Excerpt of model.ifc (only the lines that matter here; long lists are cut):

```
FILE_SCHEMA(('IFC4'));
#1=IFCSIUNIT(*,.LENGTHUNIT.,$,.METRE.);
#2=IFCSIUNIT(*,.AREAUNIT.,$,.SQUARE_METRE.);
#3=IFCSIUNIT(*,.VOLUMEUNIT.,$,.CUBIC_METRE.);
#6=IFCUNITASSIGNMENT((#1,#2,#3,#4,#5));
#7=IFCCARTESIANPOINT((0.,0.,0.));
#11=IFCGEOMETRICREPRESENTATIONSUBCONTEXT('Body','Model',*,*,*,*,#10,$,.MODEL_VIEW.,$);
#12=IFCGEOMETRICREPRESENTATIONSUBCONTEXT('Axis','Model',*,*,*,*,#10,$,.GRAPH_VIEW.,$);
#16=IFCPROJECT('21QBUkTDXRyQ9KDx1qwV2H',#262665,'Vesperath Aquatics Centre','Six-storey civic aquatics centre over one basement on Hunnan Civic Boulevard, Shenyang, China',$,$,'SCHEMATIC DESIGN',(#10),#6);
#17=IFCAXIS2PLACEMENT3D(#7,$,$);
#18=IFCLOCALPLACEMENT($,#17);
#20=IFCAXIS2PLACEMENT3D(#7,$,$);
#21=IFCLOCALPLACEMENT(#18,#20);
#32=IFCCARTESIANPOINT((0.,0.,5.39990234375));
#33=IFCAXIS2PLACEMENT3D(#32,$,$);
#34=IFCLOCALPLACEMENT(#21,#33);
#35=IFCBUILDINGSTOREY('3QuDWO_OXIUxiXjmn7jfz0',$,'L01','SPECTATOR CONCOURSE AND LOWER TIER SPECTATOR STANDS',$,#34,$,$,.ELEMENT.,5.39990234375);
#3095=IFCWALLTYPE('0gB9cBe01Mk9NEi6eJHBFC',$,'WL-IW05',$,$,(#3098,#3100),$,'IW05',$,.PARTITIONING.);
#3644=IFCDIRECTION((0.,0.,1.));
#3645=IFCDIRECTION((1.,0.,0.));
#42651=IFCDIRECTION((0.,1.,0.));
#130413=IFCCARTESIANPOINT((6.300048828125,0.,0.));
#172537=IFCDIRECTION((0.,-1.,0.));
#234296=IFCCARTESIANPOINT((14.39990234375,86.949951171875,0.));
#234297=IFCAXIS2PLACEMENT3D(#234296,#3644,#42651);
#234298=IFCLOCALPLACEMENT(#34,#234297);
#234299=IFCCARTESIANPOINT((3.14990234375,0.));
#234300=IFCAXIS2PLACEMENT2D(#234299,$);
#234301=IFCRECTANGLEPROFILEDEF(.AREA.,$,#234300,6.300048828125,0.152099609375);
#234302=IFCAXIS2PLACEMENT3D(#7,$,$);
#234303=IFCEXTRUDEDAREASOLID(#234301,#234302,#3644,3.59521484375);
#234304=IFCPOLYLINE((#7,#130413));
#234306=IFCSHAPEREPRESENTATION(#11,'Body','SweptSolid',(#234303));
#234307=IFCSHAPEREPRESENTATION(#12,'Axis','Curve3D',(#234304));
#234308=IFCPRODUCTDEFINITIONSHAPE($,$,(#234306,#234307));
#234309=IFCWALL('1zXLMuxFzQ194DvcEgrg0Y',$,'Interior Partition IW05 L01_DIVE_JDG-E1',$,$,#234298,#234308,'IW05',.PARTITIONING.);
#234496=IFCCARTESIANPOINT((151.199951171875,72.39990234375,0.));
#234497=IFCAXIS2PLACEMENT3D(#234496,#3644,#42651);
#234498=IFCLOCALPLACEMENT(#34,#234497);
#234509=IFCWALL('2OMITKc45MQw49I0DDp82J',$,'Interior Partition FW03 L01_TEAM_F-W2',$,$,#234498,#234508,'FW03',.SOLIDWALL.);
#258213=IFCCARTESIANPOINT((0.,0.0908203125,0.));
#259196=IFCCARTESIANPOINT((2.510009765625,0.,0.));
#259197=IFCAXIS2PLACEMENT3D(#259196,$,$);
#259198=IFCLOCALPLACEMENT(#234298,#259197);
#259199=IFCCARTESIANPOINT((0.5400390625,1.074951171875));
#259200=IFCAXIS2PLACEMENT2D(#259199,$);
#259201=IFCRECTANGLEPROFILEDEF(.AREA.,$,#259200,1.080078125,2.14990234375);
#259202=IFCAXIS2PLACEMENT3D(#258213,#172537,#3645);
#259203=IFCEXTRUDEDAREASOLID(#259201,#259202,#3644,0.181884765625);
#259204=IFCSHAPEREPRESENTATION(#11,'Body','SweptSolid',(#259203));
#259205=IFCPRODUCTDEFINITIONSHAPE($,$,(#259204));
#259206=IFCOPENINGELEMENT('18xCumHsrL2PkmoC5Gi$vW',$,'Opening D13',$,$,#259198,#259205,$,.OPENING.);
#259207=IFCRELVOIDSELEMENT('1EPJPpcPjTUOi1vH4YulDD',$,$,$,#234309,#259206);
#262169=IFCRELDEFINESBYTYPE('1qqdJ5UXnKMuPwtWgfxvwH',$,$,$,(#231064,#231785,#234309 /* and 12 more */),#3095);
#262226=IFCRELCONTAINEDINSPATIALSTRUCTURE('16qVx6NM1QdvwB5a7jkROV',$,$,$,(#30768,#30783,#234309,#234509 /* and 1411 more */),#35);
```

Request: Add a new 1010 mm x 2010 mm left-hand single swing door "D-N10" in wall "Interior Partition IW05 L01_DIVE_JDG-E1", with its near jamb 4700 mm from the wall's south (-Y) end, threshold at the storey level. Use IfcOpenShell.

```python
import numpy as np
import ifcopenshell
import ifcopenshell.api.feature
import ifcopenshell.api.geometry
import ifcopenshell.api.root
import ifcopenshell.api.spatial
import ifcopenshell.geom
import ifcopenshell.util.element
import ifcopenshell.util.placement
import ifcopenshell.util.representation
import ifcopenshell.util.shape
import ifcopenshell.util.unit

model = ifcopenshell.open("model.ifc")
unit_scale = ifcopenshell.util.unit.calculate_unit_scale(model)
settings = ifcopenshell.geom.settings()


def volume(element):
    """Net volume in cubic metres, openings subtracted."""
    shape = ifcopenshell.geom.create_shape(settings, element)
    return ifcopenshell.util.shape.get_volume(shape.geometry)


wall = model.by_id(234309)
storey = ifcopenshell.util.element.get_container(wall, ifc_class="IfcBuildingStorey")
context = ifcopenshell.util.representation.get_context(model, "Model", "Body", "MODEL_VIEW")
before = volume(wall)

width, height, from_end, sill = 1.01, 2.01, 4.7, 0.0  # metres

# The wall runs along its own X axis, and the end named is its -X end.
wall_shape = ifcopenshell.geom.create_shape(settings, wall)
x, y, z = ifcopenshell.util.shape.get_vertices(wall_shape.geometry).T
start = x.min() + from_end
face, thickness = float(y.min()), float(y.max() - y.min())
wall_matrix = ifcopenshell.util.placement.get_local_placement(wall.ObjectPlacement)
level = ifcopenshell.util.placement.get_local_placement(storey.ObjectPlacement)[2, 3]


def in_wall(x, y):
    """Placement at x, y metres in the wall's axes, at sill height."""
    matrix = wall_matrix.copy()
    matrix[:, 3] = wall_matrix @ np.array([x / unit_scale, y / unit_scale, 0.0, 1.0])
    matrix[2, 3] = level + sill / unit_scale
    return matrix


# Opening: a box that overshoots both wall faces by 50 mm.
opening = ifcopenshell.api.root.create_entity(model, ifc_class="IfcOpeningElement", predefined_type="OPENING")
box = ifcopenshell.api.geometry.add_wall_representation(
    model, context=context, length=width, height=height, thickness=thickness + 0.1
)
ifcopenshell.api.geometry.assign_representation(model, product=opening, representation=box)
ifcopenshell.api.geometry.edit_object_placement(model, product=opening, matrix=in_wall(start, face - 0.05), is_si=False)
ifcopenshell.api.feature.add_feature(model, feature=opening, element=wall)

door = ifcopenshell.api.root.create_entity(model, ifc_class="IfcDoor", name="D-N10", predefined_type="DOOR")
door.OverallWidth, door.OverallHeight = width / unit_scale, height / unit_scale
door.OperationType = "SINGLE_SWING_LEFT"
body = ifcopenshell.api.geometry.add_door_representation(
    model,
    context=context,
    overall_width=door.OverallWidth,
    overall_height=door.OverallHeight,
    operation_type="SINGLE_SWING_LEFT",
    lining_properties={"LiningDepth": thickness / unit_scale, "ThresholdDepth": thickness / unit_scale},
)
ifcopenshell.api.geometry.assign_representation(model, product=door, representation=body)
ifcopenshell.api.spatial.assign_container(model, products=[door], relating_structure=storey)
ifcopenshell.api.feature.add_filling(model, opening=opening, element=door)

# The lining spans the wall, so the door starts at the wall face.
ifcopenshell.api.geometry.edit_object_placement(model, product=door, matrix=in_wall(start, face), is_si=False)

after = volume(wall)

print(f"wall volume {before:.3f} -> {after:.3f} m3")

model.write("model_rev.ifc")
```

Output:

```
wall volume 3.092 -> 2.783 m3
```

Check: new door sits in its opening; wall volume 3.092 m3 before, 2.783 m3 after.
